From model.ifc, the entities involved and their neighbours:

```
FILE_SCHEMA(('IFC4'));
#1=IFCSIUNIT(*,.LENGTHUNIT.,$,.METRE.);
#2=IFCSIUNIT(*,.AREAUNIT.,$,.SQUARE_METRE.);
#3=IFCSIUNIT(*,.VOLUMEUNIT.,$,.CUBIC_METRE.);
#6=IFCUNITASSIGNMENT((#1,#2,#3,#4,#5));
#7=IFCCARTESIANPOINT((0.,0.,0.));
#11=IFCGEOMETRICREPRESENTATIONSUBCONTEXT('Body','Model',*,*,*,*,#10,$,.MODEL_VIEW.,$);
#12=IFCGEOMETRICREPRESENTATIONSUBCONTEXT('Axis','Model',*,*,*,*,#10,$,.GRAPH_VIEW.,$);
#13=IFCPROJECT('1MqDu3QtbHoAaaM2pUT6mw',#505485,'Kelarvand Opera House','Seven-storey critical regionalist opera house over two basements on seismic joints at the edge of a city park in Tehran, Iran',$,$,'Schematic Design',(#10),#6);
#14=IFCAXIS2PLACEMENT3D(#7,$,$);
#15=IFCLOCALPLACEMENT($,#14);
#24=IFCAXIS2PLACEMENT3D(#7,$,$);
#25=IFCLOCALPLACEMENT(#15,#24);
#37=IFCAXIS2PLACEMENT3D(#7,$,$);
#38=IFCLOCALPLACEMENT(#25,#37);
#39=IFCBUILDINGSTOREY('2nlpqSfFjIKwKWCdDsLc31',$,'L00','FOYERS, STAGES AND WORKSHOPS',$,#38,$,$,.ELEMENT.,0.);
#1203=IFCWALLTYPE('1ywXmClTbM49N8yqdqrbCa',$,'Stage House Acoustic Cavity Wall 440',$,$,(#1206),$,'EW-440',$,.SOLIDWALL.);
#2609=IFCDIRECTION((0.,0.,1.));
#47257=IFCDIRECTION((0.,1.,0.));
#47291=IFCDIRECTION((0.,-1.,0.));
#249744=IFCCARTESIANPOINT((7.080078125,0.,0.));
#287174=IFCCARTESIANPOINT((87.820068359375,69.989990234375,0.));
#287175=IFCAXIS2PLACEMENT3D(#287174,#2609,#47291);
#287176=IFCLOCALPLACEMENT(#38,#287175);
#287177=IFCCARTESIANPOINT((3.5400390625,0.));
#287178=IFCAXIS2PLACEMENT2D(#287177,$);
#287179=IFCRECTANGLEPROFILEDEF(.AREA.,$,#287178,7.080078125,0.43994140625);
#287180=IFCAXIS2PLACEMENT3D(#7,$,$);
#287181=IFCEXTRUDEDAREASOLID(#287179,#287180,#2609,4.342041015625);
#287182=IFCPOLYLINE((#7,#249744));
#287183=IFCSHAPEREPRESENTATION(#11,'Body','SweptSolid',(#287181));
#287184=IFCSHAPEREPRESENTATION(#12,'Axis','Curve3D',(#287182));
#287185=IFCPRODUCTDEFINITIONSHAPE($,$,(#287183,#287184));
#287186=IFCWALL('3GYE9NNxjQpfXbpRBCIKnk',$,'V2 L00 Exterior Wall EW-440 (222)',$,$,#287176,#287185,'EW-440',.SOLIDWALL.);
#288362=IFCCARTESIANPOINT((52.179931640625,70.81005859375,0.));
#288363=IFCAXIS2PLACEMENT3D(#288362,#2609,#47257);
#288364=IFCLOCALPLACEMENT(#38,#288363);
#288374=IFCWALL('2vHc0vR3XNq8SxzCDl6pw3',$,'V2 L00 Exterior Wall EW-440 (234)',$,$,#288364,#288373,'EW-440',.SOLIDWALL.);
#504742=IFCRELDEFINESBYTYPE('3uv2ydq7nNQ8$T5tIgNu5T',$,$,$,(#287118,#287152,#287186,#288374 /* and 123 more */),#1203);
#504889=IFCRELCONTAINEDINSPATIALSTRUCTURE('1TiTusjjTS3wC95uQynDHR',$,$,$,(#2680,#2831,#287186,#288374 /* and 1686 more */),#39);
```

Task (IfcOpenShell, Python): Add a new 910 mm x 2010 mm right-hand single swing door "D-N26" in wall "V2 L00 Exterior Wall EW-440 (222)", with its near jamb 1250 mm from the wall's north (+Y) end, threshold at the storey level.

```python
import numpy as np
import ifcopenshell
import ifcopenshell.api.feature
import ifcopenshell.api.geometry
import ifcopenshell.api.root
import ifcopenshell.api.spatial
import ifcopenshell.geom
import ifcopenshell.util.element
import ifcopenshell.util.placement
import ifcopenshell.util.representation
import ifcopenshell.util.shape
import ifcopenshell.util.unit

model = ifcopenshell.open("model.ifc")
unit_scale = ifcopenshell.util.unit.calculate_unit_scale(model)
settings = ifcopenshell.geom.settings()


def volume(element):
    """Net volume in cubic metres, openings subtracted."""
    shape = ifcopenshell.geom.create_shape(settings, element)
    return ifcopenshell.util.shape.get_volume(shape.geometry)


wall = model.by_id(287186)
storey = ifcopenshell.util.element.get_container(wall, ifc_class="IfcBuildingStorey")
context = ifcopenshell.util.representation.get_context(model, "Model", "Body", "MODEL_VIEW")
before = volume(wall)

width, height, from_end, sill = 0.91, 2.01, 1.25, 0.0  # metres

# The wall runs along its own X axis, and the end named is its -X end.
wall_shape = ifcopenshell.geom.create_shape(settings, wall)
x, y, z = ifcopenshell.util.shape.get_vertices(wall_shape.geometry).T
start = x.min() + from_end
face, thickness = float(y.min()), float(y.max() - y.min())
wall_matrix = ifcopenshell.util.placement.get_local_placement(wall.ObjectPlacement)
level = ifcopenshell.util.placement.get_local_placement(storey.ObjectPlacement)[2, 3]


def in_wall(x, y):
    """Placement at x, y metres in the wall's axes, at sill height."""
    matrix = wall_matrix.copy()
    matrix[:, 3] = wall_matrix @ np.array([x / unit_scale, y / unit_scale, 0.0, 1.0])
    matrix[2, 3] = level + sill / unit_scale
    return matrix


# Opening: a box that overshoots both wall faces by 50 mm.
opening = ifcopenshell.api.root.create_entity(model, ifc_class="IfcOpeningElement", predefined_type="OPENING")
box = ifcopenshell.api.geometry.add_wall_representation(
    model, context=context, length=width, height=height, thickness=thickness + 0.1
)
ifcopenshell.api.geometry.assign_representation(model, product=opening, representation=box)
ifcopenshell.api.geometry.edit_object_placement(model, product=opening, matrix=in_wall(start, face - 0.05), is_si=False)
ifcopenshell.api.feature.add_feature(model, feature=opening, element=wall)

door = ifcopenshell.api.root.create_entity(model, ifc_class="IfcDoor", name="D-N26", predefined_type="DOOR")
door.OverallWidth, door.OverallHeight = width / unit_scale, height / unit_scale
door.OperationType = "SINGLE_SWING_RIGHT"
body = ifcopenshell.api.geometry.add_door_representation(
    model,
    context=context,
    overall_width=door.OverallWidth,
    overall_height=door.OverallHeight,
    operation_type="SINGLE_SWING_RIGHT",
    lining_properties={"LiningDepth": thickness / unit_scale, "ThresholdDepth": thickness / unit_scale},
)
ifcopenshell.api.geometry.assign_representation(model, product=door, representation=body)
ifcopenshell.api.spatial.assign_container(model, products=[door], relating_structure=storey)
ifcopenshell.api.feature.add_filling(model, opening=opening, element=door)

# The lining spans the wall, so the door starts at the wall face.
ifcopenshell.api.geometry.edit_object_placement(model, product=door, matrix=in_wall(start, face), is_si=False)

after = volume(wall)

print(f"wall volume {before:.3f} -> {after:.3f} m3")

model.write("model_v2.ifc")
```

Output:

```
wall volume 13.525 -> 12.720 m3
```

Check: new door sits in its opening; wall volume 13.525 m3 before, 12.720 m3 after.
